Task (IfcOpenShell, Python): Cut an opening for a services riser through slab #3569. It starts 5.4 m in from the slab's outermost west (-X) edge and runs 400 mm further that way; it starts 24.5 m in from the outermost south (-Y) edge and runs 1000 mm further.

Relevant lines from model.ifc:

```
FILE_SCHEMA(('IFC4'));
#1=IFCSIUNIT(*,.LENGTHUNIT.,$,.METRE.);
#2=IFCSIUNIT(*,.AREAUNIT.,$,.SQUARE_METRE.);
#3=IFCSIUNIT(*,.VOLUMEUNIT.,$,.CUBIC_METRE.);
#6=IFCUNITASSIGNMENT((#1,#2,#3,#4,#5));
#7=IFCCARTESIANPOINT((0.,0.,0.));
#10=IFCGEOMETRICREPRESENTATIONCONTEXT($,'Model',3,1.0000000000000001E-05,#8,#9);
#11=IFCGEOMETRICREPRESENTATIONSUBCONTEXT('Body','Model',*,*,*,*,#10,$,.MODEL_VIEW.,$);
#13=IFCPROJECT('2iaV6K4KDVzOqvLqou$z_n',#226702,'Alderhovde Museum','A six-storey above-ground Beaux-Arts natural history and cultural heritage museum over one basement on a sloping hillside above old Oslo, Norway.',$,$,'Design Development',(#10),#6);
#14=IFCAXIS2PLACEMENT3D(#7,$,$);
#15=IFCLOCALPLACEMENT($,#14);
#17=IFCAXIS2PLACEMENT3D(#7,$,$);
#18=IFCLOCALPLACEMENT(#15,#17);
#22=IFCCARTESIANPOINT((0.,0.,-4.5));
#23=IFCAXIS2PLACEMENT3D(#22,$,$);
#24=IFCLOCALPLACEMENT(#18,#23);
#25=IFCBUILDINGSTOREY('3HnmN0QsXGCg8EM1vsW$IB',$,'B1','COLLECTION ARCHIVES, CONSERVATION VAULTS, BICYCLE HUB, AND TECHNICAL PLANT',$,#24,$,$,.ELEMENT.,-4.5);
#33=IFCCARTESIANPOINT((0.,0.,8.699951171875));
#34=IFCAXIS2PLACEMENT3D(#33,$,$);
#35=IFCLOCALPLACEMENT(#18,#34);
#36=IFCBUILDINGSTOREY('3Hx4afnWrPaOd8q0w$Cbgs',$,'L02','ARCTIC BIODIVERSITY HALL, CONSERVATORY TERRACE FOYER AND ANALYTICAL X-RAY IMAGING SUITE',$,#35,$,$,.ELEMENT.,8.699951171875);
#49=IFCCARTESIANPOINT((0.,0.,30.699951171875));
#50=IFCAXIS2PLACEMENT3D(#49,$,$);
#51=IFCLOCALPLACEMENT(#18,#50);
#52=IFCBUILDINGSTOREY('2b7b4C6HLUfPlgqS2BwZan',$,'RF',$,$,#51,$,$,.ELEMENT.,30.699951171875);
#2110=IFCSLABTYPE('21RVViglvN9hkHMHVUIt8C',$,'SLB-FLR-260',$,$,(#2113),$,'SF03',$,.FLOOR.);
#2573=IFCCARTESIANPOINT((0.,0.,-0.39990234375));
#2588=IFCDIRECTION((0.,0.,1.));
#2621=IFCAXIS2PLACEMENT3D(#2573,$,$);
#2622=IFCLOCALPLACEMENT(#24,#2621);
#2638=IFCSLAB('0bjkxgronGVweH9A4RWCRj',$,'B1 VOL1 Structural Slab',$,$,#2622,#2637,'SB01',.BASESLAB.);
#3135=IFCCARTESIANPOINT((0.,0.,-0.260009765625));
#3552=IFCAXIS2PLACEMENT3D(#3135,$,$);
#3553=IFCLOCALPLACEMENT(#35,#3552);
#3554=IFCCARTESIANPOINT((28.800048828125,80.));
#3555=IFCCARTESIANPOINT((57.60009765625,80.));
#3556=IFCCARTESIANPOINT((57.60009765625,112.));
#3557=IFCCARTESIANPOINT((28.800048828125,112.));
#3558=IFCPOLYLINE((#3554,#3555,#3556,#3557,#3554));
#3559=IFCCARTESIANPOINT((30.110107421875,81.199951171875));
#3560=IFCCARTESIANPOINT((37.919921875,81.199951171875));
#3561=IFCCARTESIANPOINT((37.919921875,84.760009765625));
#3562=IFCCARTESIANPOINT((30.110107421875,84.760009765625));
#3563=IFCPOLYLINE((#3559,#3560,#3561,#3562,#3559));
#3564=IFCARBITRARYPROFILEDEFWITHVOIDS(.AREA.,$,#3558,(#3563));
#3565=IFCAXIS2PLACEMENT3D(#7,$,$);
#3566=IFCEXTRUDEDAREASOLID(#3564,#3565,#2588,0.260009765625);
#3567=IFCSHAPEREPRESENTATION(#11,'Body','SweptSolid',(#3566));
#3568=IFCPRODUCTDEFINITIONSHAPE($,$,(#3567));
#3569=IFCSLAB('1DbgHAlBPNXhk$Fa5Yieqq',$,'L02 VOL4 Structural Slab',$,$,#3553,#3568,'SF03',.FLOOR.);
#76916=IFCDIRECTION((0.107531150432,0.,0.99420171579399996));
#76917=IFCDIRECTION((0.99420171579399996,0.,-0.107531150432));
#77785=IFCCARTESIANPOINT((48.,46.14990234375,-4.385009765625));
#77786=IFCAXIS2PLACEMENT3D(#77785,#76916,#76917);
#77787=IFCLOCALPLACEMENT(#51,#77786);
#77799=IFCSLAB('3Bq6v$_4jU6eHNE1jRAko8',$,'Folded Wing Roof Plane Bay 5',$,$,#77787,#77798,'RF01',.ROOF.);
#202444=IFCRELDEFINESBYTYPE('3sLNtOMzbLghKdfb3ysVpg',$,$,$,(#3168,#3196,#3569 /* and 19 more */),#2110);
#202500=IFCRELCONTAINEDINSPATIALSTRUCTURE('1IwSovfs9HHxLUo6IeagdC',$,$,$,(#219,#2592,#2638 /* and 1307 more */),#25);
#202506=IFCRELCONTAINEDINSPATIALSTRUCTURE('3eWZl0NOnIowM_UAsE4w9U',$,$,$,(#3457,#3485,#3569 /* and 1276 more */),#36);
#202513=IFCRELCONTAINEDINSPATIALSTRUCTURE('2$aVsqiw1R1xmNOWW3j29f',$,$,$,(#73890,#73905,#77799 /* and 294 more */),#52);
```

```python
import numpy as np
import ifcopenshell
import ifcopenshell.api.feature
import ifcopenshell.api.geometry
import ifcopenshell.api.root
import ifcopenshell.geom
import ifcopenshell.util.placement
import ifcopenshell.util.representation
import ifcopenshell.util.shape
import ifcopenshell.util.unit

model = ifcopenshell.open("model.ifc")
unit_scale = ifcopenshell.util.unit.calculate_unit_scale(model)
settings = ifcopenshell.geom.settings()


def volume(element):
    """Net volume in cubic metres, openings subtracted."""
    shape = ifcopenshell.geom.create_shape(settings, element)
    return ifcopenshell.util.shape.get_volume(shape.geometry)


slab = model.by_guid("1DbgHAlBPNXhk$Fa5Yieqq")
before = volume(slab)

# Extent in the slab's own axes, in metres. The edges named are its -X and -Y sides.
slab_shape = ifcopenshell.geom.create_shape(settings, slab)
vertices = ifcopenshell.util.shape.get_vertices(slab_shape.geometry)
x_min, y_min, bottom = vertices.min(axis=0)
top = vertices[:, 2].max()

opening = ifcopenshell.api.root.create_entity(model, ifc_class="IfcOpeningElement", name="Services riser opening", predefined_type="OPENING")
context = ifcopenshell.util.representation.get_context(model, "Model", "Body", "MODEL_VIEW")
width, depth = 0.4, 1
outline = [(0.0, 0.0), (width, 0.0), (width, depth), (0.0, depth), (0.0, 0.0)]
# Overshoot both faces by 50 mm so the cut is clean.
shape = ifcopenshell.api.geometry.add_slab_representation(
    model, context=context, depth=top - bottom + 0.1, polyline=outline
)
ifcopenshell.api.geometry.assign_representation(model, product=opening, representation=shape)

matrix = ifcopenshell.util.placement.get_local_placement(slab.ObjectPlacement)
matrix[:, 3] = matrix @ np.append(np.array([x_min + 5.4, y_min + 24.5, bottom - 0.05]) / unit_scale, 1.0)
ifcopenshell.api.geometry.edit_object_placement(model, product=opening, matrix=matrix, is_si=False)
ifcopenshell.api.feature.add_feature(model, feature=opening, element=slab)

after = volume(slab)

print(f"slab volume {before:.3f} -> {after:.3f} m3")

model.write("model_updated.ifc")
```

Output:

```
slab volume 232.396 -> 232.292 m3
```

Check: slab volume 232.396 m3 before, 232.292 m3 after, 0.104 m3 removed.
